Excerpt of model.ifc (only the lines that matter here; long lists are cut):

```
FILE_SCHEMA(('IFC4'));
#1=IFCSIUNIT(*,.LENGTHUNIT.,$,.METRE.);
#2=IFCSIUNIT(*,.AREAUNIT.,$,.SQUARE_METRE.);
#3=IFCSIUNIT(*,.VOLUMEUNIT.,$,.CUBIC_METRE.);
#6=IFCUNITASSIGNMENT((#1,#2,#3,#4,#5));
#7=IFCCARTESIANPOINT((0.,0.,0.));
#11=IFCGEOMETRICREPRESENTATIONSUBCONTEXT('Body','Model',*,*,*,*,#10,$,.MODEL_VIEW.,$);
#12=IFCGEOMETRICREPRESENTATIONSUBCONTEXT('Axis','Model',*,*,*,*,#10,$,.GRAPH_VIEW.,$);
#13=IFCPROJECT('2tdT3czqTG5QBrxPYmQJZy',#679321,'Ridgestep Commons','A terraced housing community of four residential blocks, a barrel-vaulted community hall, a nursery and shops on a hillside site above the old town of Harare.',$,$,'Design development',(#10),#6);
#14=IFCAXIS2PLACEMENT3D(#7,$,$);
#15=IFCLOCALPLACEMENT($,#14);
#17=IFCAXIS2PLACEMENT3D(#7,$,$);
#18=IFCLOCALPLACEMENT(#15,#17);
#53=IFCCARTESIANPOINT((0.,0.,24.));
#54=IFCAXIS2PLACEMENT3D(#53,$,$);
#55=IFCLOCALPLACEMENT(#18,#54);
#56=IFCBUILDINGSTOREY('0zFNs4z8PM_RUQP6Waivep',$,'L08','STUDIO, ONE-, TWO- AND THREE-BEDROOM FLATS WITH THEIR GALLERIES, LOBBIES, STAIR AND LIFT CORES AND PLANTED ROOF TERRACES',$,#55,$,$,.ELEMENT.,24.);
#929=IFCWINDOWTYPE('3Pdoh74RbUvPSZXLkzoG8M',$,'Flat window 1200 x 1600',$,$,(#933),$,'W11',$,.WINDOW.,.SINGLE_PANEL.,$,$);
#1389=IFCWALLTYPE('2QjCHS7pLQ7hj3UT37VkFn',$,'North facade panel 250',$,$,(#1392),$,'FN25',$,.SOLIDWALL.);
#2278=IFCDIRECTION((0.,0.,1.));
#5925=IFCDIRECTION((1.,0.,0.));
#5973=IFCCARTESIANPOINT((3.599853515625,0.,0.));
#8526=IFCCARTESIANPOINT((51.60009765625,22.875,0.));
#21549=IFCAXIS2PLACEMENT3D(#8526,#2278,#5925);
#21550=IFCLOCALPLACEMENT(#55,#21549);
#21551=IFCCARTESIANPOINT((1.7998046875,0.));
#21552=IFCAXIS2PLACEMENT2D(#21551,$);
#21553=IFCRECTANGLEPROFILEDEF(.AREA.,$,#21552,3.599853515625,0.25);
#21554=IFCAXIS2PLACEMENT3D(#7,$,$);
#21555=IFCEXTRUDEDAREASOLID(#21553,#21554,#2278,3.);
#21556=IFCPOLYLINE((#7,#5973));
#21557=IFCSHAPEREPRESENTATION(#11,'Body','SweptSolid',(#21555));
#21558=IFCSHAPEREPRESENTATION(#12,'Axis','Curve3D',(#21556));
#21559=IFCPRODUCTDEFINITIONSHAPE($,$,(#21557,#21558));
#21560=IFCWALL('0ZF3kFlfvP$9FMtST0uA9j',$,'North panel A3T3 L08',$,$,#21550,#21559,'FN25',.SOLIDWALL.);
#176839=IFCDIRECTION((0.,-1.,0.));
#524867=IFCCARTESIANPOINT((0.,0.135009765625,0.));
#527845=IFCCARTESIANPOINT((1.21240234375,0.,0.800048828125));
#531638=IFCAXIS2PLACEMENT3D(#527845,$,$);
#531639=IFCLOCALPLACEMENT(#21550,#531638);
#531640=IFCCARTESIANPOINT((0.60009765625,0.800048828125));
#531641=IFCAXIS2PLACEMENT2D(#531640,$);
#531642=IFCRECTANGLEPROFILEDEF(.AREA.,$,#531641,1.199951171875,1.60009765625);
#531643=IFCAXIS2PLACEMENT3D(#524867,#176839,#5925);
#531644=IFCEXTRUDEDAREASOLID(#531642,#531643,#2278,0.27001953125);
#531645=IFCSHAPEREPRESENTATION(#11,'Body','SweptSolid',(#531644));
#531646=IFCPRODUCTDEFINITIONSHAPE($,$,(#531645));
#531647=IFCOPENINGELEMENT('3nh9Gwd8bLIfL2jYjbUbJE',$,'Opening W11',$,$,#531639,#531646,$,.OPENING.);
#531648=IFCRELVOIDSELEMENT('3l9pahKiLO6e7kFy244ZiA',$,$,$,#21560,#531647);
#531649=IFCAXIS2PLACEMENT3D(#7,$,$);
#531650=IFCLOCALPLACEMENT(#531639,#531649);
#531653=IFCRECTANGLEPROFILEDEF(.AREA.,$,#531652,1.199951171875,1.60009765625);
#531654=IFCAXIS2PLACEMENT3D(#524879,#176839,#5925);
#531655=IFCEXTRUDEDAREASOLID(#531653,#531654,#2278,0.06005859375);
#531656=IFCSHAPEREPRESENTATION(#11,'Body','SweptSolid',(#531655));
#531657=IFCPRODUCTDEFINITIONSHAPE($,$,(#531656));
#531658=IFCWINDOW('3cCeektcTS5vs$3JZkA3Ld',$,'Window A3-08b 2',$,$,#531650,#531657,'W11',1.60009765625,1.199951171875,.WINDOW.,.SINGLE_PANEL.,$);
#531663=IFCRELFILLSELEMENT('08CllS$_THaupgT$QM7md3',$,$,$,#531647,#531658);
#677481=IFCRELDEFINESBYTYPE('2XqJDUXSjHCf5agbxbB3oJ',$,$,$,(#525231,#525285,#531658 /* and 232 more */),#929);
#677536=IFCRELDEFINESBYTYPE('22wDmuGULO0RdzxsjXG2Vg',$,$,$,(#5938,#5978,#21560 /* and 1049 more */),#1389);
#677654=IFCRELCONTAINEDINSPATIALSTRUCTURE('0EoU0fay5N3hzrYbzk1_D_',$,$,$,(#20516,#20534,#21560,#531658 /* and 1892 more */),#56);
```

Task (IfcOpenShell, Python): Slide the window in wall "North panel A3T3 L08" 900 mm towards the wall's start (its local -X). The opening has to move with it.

```python
import ifcopenshell
import ifcopenshell.api.geometry
import ifcopenshell.util.placement
import ifcopenshell.util.unit

model = ifcopenshell.open("model.ifc")
unit_scale = ifcopenshell.util.unit.calculate_unit_scale(model)

window = model.by_guid("3cCeektcTS5vs$3JZkA3Ld")
opening = window.FillsVoids[0].RelatingOpeningElement
wall = opening.VoidsElements[0].RelatingBuildingElement

wall_matrix = ifcopenshell.util.placement.get_local_placement(wall.ObjectPlacement)
shift = wall_matrix[:3, 0] * -0.9 / unit_scale
before = ifcopenshell.util.placement.get_local_placement(window.ObjectPlacement)[:3, 3].copy()

# The window is placed relative to its opening, so it follows when the opening moves.
matrix = ifcopenshell.util.placement.get_local_placement(opening.ObjectPlacement)
matrix[:3, 3] += shift
ifcopenshell.api.geometry.edit_object_placement(
    model, product=opening, matrix=matrix, is_si=False, should_transform_children=True
)

after = ifcopenshell.util.placement.get_local_placement(window.ObjectPlacement)[:3, 3]
print("window moved by", (after - before).round(3) + 0.0)

model.write("model-out.ifc")
```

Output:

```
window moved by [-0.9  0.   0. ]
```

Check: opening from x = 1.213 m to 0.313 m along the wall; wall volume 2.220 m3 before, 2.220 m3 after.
